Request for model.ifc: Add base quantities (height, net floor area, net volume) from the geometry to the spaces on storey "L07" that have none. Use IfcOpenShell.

First a look at what the model holds.

```python
import ifcopenshell
import ifcopenshell.util.element
import ifcopenshell.util.unit

model = ifcopenshell.open("model.ifc")
print(model.schema)
for unit_type in ("LENGTHUNIT", "AREAUNIT", "VOLUMEUNIT"):
    print(unit_type, ifcopenshell.util.unit.calculate_unit_scale(model, unit_type))
storey = next(s for s in model.by_type("IfcBuildingStorey") if s.Name == "L07")
spaces = [e for e in ifcopenshell.util.element.get_decomposition(storey) if e.is_a("IfcSpace")]
for e in sorted(spaces, key=lambda e: e.id()):
    print(e.id(), e.is_a(), e.Name, list(ifcopenshell.util.element.get_psets(e, qtos_only=True)), sep=" | ")
```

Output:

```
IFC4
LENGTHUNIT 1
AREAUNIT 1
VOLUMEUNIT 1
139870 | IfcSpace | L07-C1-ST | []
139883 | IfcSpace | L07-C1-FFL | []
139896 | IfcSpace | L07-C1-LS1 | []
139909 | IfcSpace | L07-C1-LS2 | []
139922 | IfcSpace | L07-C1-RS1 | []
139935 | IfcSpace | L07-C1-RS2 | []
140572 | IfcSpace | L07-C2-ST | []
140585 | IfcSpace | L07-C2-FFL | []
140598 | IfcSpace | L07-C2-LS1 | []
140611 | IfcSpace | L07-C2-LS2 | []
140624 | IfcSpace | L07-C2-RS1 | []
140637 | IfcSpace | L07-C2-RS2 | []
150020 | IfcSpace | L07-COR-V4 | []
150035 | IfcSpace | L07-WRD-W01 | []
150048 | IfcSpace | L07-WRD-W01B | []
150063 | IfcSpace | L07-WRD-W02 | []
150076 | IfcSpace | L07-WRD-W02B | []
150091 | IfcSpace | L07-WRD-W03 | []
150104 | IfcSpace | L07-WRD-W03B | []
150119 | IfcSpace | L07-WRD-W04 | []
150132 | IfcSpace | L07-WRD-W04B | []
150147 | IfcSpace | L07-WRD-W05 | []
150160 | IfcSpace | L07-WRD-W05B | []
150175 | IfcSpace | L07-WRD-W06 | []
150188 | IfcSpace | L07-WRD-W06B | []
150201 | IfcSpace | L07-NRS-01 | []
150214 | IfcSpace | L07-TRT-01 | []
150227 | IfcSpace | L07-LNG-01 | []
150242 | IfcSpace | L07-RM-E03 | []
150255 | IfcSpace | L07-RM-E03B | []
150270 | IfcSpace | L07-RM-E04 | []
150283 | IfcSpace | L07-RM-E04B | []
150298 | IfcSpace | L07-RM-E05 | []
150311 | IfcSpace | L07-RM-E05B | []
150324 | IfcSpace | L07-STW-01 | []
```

```python
import ifcopenshell
import ifcopenshell.api.pset
import ifcopenshell.geom
import ifcopenshell.util.element
import ifcopenshell.util.shape
import ifcopenshell.util.unit

model = ifcopenshell.open("model.ifc")
unit_scale = ifcopenshell.util.unit.calculate_unit_scale(model)
area_scale = ifcopenshell.util.unit.calculate_unit_scale(model, "AREAUNIT")
volume_scale = ifcopenshell.util.unit.calculate_unit_scale(model, "VOLUMEUNIT")
settings = ifcopenshell.geom.settings()

storey = next(s for s in model.by_type("IfcBuildingStorey") if s.Name == "L07")
spaces = [e for e in ifcopenshell.util.element.get_decomposition(storey) if e.is_a("IfcSpace")]

for e in sorted(spaces, key=lambda e: e.id()):
    if ifcopenshell.util.element.get_psets(e, qtos_only=True, should_inherit=False):
        continue
    # Geometry comes back in metres, in the element's own axes.
    shape = ifcopenshell.geom.create_shape(settings, e)
    values = {
        "Height": ifcopenshell.util.shape.get_z(shape.geometry) / unit_scale,
        "NetFloorArea": ifcopenshell.util.shape.get_footprint_area(shape.geometry) / area_scale,
        "NetVolume": ifcopenshell.util.shape.get_volume(shape.geometry) / volume_scale,
    }
    qto = ifcopenshell.api.pset.add_qto(model, product=e, name="Qto_SpaceBaseQuantities")
    ifcopenshell.api.pset.edit_qto(model, qto=qto, properties=values)
    print(e.id(), {k: round(v, 3) for k, v in values.items()})

model.write("model_rev.ifc")
```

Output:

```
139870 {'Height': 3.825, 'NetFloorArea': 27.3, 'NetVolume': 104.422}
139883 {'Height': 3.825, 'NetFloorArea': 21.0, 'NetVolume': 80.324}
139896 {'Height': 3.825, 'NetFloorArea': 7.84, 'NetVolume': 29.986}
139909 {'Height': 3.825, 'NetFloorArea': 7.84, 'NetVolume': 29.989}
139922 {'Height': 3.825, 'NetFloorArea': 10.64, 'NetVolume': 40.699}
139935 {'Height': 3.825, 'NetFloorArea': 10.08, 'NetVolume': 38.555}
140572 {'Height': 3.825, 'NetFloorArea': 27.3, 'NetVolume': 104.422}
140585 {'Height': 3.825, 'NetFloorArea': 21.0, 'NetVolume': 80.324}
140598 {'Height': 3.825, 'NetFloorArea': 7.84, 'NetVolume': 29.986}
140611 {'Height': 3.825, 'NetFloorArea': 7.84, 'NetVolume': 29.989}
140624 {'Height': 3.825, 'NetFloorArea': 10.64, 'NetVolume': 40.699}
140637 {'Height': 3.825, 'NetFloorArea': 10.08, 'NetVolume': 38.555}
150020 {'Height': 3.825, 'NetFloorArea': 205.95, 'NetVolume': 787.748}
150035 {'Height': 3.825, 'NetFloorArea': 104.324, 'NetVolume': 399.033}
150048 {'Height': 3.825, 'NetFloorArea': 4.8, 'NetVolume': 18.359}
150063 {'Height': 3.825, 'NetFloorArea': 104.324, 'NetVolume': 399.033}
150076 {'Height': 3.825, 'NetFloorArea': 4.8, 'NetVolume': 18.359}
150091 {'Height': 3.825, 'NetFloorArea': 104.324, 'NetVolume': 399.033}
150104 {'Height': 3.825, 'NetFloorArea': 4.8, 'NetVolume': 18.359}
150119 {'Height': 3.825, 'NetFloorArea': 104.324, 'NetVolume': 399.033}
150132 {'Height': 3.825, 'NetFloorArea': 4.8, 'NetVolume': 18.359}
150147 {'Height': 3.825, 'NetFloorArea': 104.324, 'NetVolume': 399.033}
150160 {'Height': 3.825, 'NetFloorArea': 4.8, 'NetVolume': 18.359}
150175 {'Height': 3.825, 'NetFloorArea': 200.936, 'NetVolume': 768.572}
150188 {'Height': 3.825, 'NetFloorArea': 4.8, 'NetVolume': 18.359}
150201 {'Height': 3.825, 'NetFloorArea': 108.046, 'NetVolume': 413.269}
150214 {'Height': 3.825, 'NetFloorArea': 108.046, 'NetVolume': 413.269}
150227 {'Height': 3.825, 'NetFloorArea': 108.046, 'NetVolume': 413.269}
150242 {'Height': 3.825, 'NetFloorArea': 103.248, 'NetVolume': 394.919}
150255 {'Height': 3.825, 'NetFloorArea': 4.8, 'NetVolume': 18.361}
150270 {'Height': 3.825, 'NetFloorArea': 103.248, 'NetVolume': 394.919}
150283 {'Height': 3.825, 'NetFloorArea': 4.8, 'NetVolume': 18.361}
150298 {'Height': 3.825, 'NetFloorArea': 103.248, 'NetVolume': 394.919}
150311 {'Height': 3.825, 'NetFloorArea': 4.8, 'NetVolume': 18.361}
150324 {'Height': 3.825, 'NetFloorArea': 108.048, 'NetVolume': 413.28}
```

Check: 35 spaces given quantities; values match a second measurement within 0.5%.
